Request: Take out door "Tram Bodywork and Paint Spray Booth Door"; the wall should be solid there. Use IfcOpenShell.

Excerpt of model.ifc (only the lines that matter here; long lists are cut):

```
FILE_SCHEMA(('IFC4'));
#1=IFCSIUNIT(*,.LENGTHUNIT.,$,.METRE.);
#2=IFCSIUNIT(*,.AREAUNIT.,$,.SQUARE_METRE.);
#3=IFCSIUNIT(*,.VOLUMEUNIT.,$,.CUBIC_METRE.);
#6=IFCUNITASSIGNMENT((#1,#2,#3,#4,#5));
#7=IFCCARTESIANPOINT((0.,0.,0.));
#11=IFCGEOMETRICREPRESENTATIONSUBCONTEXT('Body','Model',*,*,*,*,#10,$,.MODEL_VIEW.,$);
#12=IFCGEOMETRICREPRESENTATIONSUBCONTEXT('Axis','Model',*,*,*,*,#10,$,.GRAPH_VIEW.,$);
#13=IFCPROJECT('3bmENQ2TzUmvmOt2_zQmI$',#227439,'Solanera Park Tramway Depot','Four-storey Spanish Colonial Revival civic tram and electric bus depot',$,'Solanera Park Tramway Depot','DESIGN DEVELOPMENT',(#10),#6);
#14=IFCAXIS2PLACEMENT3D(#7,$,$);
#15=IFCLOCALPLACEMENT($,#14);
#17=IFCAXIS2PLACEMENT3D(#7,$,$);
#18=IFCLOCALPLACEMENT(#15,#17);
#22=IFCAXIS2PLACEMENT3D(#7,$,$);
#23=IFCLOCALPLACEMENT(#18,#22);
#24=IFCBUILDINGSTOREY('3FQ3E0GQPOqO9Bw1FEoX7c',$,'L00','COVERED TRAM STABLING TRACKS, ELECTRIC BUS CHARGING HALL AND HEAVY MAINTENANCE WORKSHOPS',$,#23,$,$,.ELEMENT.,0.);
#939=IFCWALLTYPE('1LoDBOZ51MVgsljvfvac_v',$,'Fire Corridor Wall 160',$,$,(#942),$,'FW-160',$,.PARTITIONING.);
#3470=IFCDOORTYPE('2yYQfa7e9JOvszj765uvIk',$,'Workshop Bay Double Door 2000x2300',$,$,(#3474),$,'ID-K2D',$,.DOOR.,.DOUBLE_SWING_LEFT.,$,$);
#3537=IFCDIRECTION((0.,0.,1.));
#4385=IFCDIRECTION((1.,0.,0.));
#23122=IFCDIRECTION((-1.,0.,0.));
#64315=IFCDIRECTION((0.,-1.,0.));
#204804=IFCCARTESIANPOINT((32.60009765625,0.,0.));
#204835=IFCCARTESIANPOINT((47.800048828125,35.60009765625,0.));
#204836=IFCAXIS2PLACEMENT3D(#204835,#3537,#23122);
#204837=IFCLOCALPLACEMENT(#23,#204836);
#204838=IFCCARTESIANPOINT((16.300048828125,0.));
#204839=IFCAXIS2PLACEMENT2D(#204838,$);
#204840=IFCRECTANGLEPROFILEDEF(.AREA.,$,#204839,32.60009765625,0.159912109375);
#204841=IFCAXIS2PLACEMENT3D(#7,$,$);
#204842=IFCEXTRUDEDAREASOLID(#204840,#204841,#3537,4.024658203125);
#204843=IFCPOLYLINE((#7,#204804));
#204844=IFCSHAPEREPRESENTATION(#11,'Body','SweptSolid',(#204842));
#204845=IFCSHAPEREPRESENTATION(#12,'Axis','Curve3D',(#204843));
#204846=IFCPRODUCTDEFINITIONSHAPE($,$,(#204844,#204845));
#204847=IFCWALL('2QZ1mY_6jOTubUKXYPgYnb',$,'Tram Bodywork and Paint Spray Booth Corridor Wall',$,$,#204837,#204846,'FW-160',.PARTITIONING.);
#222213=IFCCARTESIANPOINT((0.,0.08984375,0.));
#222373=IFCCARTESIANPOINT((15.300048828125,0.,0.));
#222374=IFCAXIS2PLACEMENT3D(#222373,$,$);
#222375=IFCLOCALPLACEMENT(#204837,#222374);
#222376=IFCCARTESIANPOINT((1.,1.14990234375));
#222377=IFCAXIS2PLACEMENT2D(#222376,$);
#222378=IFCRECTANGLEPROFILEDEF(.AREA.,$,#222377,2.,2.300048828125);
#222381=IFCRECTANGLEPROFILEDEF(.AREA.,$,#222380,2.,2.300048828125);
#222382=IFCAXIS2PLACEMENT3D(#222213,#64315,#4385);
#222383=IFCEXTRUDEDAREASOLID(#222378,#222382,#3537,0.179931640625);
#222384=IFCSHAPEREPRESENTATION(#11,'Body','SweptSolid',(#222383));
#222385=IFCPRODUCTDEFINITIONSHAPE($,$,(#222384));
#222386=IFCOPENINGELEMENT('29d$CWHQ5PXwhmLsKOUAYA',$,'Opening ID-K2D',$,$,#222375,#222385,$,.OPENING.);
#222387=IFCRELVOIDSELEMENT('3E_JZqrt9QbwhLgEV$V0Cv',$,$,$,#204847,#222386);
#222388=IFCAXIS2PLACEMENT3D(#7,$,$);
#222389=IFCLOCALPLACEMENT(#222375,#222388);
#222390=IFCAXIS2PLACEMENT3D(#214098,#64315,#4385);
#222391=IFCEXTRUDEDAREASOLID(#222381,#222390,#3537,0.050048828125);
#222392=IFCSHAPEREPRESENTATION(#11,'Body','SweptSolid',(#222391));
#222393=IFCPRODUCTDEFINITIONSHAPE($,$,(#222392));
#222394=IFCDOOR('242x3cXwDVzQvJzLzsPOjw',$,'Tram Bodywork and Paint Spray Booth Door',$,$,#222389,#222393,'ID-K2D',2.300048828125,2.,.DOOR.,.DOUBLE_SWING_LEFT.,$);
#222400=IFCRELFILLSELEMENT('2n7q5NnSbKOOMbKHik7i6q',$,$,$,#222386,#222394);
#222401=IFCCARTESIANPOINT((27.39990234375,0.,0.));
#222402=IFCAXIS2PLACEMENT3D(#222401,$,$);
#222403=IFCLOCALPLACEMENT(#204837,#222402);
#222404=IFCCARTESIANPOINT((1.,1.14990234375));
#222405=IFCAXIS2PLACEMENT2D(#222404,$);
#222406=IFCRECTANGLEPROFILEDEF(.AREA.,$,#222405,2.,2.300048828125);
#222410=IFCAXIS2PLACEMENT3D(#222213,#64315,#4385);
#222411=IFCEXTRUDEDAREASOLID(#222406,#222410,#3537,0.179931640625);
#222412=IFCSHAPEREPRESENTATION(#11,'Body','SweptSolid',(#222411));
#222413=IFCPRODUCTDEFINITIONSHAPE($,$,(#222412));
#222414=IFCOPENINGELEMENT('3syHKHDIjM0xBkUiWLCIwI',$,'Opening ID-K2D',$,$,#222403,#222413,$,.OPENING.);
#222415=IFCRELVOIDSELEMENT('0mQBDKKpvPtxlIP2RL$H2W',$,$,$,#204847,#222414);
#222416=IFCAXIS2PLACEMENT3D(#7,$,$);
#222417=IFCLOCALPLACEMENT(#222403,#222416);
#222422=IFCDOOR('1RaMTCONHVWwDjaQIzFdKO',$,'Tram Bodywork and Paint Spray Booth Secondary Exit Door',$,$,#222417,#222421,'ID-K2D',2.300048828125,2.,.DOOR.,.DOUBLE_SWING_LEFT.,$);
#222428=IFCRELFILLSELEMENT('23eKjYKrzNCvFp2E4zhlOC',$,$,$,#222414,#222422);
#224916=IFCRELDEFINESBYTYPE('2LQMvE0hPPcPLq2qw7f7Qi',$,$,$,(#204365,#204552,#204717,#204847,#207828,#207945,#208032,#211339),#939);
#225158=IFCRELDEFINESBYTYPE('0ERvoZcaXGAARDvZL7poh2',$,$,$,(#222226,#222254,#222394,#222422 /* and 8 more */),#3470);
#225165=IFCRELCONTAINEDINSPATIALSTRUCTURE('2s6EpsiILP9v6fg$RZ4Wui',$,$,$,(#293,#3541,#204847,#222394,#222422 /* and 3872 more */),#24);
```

```python
import ifcopenshell
import ifcopenshell.api.feature
import ifcopenshell.api.root
import ifcopenshell.geom
import ifcopenshell.util.shape

model = ifcopenshell.open("model.ifc")
settings = ifcopenshell.geom.settings()


def volume(element):
    """Net volume in cubic metres, openings subtracted."""
    shape = ifcopenshell.geom.create_shape(settings, element)
    return ifcopenshell.util.shape.get_volume(shape.geometry)


door = model.by_id(222394)
opening = door.FillsVoids[0].RelatingOpeningElement
wall = opening.VoidsElements[0].RelatingBuildingElement
before = volume(wall)

ifcopenshell.api.root.remove_product(model, product=door)
ifcopenshell.api.feature.remove_feature(model, feature=opening)

after = volume(wall)

print(f"wall volume {before:.3f} -> {after:.3f} m3")

model.write("model_rev.ifc")
```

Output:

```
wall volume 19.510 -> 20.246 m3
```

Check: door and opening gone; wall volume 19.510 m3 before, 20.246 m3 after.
